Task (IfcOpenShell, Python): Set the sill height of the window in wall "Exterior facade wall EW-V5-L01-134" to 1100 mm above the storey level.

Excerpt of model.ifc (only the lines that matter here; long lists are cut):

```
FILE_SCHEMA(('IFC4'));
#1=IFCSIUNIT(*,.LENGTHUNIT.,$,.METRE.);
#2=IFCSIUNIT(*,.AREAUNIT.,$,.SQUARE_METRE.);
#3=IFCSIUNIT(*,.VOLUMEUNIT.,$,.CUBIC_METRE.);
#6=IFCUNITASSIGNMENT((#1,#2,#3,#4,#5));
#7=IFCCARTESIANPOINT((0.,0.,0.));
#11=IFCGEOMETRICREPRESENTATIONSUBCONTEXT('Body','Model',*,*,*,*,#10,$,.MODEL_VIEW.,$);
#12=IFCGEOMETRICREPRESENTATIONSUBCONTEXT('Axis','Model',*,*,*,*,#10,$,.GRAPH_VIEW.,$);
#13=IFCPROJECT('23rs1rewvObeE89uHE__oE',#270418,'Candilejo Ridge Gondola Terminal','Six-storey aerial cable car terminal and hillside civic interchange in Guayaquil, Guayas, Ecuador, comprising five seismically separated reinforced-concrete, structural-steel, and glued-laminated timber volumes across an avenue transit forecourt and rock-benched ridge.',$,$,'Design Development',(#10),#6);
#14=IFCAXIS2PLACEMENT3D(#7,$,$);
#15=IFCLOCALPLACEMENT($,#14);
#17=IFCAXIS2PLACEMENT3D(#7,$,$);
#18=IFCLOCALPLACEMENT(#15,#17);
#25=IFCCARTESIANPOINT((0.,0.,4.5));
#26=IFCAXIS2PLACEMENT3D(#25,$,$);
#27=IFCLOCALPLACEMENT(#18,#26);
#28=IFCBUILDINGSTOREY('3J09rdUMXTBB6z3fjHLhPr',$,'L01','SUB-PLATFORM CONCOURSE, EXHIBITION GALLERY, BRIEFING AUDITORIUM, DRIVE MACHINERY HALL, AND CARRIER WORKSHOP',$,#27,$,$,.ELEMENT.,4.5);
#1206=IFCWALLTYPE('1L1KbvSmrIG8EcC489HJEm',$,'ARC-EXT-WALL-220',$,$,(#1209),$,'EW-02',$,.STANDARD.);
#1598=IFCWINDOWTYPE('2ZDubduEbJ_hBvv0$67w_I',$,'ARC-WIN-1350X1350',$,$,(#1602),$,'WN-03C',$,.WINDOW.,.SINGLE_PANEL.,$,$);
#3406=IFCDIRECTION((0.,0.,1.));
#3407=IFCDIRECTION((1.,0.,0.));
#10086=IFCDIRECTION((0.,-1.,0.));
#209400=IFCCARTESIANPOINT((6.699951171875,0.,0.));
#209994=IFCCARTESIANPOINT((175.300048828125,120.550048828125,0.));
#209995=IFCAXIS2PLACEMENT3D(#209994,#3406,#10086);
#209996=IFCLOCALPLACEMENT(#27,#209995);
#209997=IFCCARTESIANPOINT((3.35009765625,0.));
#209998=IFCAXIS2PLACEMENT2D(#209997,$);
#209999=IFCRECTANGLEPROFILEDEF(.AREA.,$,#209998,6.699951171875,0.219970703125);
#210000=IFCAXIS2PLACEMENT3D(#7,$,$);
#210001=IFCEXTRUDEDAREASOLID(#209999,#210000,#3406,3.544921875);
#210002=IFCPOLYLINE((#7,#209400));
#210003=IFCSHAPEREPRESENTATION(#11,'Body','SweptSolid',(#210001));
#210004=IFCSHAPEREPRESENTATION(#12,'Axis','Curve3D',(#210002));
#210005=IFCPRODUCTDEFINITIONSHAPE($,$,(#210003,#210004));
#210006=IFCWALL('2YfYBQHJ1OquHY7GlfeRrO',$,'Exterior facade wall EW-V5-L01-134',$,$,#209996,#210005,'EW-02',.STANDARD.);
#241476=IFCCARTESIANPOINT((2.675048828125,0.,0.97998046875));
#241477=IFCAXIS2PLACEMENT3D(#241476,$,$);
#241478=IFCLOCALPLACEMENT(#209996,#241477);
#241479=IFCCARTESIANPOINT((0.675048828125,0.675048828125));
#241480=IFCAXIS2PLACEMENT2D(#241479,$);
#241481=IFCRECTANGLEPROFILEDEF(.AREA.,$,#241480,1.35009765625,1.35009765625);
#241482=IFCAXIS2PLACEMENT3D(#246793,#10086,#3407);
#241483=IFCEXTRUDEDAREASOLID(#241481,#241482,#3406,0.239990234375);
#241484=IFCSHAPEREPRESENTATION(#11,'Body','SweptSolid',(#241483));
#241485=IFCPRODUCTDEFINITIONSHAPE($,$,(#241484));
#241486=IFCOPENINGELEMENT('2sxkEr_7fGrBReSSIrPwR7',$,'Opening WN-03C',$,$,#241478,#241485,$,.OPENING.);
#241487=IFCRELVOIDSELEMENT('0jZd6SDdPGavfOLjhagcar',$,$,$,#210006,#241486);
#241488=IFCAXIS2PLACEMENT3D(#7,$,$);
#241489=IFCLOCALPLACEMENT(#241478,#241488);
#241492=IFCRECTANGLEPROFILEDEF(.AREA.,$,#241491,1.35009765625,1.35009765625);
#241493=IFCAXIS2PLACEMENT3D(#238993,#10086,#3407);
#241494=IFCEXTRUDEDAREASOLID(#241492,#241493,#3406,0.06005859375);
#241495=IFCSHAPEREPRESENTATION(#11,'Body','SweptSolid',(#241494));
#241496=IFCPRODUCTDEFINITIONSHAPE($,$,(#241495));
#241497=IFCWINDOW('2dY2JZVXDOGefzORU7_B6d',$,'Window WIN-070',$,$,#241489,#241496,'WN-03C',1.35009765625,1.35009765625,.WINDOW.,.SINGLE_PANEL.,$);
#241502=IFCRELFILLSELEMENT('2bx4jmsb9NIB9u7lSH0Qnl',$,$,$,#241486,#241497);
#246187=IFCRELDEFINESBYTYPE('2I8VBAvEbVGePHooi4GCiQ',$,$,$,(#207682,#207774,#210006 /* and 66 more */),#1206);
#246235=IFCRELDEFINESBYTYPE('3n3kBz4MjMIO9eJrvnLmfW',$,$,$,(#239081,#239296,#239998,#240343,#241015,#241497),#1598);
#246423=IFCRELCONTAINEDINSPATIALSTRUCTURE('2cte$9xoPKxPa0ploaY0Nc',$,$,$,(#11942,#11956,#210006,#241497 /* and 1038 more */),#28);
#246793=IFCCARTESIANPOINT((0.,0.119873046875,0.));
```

```python
import numpy as np
import ifcopenshell
import ifcopenshell.api.geometry
import ifcopenshell.geom
import ifcopenshell.util.element
import ifcopenshell.util.placement
import ifcopenshell.util.shape
import ifcopenshell.util.unit

model = ifcopenshell.open("model.ifc")
unit_scale = ifcopenshell.util.unit.calculate_unit_scale(model)

window = model.by_guid("2dY2JZVXDOGefzORU7_B6d")
opening = window.FillsVoids[0].RelatingOpeningElement
storey = ifcopenshell.util.element.get_container(window, ifc_class="IfcBuildingStorey")
level = ifcopenshell.util.placement.get_local_placement(storey.ObjectPlacement)[2, 3]

# The opening's origin need not be at the sill, so measure its lowest point.
shape = ifcopenshell.geom.create_shape(ifcopenshell.geom.settings(), opening)
bottom = ifcopenshell.util.shape.get_shape_bottom_elevation(shape, shape.geometry) / unit_scale
dz = level + 1.1 - bottom

shift = np.array([0.0, 0.0, dz])
# The window is placed relative to its opening, so it follows when the opening moves.
matrix = ifcopenshell.util.placement.get_local_placement(opening.ObjectPlacement)
matrix[:3, 3] += shift
ifcopenshell.api.geometry.edit_object_placement(
    model, product=opening, matrix=matrix, is_si=False, should_transform_children=True
)

print(f"moved by {dz * unit_scale:+.3f} m")

model.write("model_edited.ifc")
```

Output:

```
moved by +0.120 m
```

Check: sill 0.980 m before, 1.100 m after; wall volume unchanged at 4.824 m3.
